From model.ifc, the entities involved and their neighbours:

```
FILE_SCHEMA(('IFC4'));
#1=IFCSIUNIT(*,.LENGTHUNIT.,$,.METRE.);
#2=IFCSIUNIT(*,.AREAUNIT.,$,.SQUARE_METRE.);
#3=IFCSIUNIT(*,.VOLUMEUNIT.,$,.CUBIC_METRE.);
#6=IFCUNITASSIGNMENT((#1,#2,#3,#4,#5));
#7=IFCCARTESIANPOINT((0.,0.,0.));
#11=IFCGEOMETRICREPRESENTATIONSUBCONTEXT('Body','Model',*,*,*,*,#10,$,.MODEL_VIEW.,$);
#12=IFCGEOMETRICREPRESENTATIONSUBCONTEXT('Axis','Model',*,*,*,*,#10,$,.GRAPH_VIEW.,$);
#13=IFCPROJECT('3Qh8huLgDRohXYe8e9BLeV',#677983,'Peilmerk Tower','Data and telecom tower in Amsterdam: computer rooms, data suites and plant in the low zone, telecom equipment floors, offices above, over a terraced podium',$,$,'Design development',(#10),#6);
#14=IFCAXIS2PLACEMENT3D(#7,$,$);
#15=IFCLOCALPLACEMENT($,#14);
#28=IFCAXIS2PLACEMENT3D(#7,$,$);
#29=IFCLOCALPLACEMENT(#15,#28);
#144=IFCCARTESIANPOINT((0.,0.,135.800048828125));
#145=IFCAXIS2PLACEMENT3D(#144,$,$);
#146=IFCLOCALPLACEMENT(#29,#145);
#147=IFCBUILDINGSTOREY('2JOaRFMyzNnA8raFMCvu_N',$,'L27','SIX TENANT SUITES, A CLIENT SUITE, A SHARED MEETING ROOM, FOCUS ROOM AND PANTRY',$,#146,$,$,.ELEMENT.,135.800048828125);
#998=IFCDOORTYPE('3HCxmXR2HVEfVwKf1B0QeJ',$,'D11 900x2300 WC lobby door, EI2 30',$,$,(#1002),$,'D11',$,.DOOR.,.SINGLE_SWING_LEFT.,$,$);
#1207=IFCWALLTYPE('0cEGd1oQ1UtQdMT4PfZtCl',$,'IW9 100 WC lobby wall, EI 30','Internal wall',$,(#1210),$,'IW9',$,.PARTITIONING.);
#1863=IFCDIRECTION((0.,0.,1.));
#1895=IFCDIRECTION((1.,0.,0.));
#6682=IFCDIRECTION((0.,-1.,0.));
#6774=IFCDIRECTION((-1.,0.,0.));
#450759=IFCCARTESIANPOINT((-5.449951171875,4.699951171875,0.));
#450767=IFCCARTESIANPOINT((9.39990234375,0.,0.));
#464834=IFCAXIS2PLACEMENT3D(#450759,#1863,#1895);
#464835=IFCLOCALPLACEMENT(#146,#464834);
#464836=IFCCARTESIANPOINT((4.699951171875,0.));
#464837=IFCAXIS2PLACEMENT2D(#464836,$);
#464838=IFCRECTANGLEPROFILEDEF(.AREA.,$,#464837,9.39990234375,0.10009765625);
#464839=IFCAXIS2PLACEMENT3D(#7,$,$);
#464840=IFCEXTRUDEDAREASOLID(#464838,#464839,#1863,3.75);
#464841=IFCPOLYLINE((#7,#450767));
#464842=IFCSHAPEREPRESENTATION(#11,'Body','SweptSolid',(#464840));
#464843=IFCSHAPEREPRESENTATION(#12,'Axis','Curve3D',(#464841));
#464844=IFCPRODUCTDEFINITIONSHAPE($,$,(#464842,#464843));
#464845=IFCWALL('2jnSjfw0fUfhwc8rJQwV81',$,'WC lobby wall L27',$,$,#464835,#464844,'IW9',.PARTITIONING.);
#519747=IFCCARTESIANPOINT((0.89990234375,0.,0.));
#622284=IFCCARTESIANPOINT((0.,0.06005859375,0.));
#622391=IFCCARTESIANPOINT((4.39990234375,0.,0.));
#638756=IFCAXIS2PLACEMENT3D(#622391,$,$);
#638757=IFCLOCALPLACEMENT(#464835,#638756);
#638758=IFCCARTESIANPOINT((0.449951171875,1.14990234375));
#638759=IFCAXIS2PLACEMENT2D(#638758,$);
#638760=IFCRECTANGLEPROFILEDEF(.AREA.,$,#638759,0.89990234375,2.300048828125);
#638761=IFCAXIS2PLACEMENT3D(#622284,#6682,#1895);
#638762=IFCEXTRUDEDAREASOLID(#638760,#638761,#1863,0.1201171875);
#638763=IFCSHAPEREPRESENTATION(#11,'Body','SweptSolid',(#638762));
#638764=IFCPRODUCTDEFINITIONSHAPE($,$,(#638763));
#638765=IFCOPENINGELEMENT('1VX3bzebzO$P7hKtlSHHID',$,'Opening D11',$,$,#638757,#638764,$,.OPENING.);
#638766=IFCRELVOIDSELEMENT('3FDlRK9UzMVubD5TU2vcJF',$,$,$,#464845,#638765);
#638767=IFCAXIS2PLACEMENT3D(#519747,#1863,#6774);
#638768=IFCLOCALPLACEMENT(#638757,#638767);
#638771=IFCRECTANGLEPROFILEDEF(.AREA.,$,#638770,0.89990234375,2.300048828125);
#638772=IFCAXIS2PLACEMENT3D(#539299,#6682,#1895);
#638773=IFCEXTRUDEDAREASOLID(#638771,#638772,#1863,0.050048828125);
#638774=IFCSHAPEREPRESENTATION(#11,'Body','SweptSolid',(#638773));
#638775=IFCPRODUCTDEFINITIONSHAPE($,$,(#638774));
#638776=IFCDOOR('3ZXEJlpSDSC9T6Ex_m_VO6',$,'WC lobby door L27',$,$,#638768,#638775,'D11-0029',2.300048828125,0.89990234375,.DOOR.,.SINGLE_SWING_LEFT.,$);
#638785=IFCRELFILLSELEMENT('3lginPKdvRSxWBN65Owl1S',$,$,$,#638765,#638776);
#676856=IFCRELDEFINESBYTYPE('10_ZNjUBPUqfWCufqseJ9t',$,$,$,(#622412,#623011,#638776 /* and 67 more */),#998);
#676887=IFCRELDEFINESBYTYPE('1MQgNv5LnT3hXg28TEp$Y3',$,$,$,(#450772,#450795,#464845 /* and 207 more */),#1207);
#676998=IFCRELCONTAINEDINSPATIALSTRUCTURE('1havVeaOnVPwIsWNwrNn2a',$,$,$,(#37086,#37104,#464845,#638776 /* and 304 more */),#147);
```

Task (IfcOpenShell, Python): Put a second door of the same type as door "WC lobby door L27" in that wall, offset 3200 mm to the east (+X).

```python
import ifcopenshell
import ifcopenshell.api.feature
import ifcopenshell.api.geometry
import ifcopenshell.api.root
import ifcopenshell.geom
import ifcopenshell.util.element
import ifcopenshell.util.placement
import ifcopenshell.util.shape

model = ifcopenshell.open("model.ifc")
settings = ifcopenshell.geom.settings()


def volume(element):
    """Net volume in cubic metres, openings subtracted."""
    shape = ifcopenshell.geom.create_shape(settings, element)
    return ifcopenshell.util.shape.get_volume(shape.geometry)


door = model.by_guid("3ZXEJlpSDSC9T6Ex_m_VO6")
opening = door.FillsVoids[0].RelatingOpeningElement
wall = opening.VoidsElements[0].RelatingBuildingElement
before = volume(wall)
shift = ifcopenshell.util.placement.get_local_placement(wall.ObjectPlacement)[:3, 0] * 3.2

# copy_class copies the void relationship, type, container and properties, but no geometry.
new_opening = ifcopenshell.api.root.copy_class(model, product=opening)
new_opening.Representation = ifcopenshell.util.element.copy_deep(
    model, opening.Representation, exclude=["IfcGeometricRepresentationContext", "IfcRepresentationMap"]
)
new_door = ifcopenshell.api.root.copy_class(model, product=door)
new_door.Representation = ifcopenshell.util.element.copy_deep(
    model, door.Representation, exclude=["IfcGeometricRepresentationContext", "IfcRepresentationMap"]
)
new_door.Tag = None
ifcopenshell.api.feature.add_filling(model, opening=new_opening, element=new_door)

for old, new in ((opening, new_opening), (door, new_door)):
    matrix = ifcopenshell.util.placement.get_local_placement(old.ObjectPlacement)
    matrix[:3, 3] += shift
    ifcopenshell.api.geometry.edit_object_placement(model, product=new, matrix=matrix, is_si=False)

after = volume(wall)

print(f"wall volume {before:.3f} -> {after:.3f} m3")

model.write("model_updated.ifc")
```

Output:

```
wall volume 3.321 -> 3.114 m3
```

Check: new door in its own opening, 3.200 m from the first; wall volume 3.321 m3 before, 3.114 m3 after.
